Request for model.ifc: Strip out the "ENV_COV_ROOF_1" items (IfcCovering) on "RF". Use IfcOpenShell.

First a look at what the model holds.

```python
import ifcopenshell
import ifcopenshell.util.element

model = ifcopenshell.open("model.ifc")
print(model.schema)
storey = next(s for s in model.by_type("IfcBuildingStorey") if s.Name == "RF")
coverings = [e for e in ifcopenshell.util.element.get_decomposition(storey) if e.is_a("IfcCovering")]
seen = {}
for e in coverings:
    element_type = ifcopenshell.util.element.get_type(e)
    name = element_type.Name if element_type not in (None, e) else None
    seen[name] = seen.get(name, 0) + 1
for name, count in sorted(seen.items(), key=str):
    print(count, "x", name)
```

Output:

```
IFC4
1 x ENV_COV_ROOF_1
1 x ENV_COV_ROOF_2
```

```python
import ifcopenshell
import ifcopenshell.api.root
import ifcopenshell.util.element

model = ifcopenshell.open("model.ifc")

storey = next(s for s in model.by_type("IfcBuildingStorey") if s.Name == "RF")
coverings = [e for e in ifcopenshell.util.element.get_decomposition(storey) if e.is_a("IfcCovering")]
targets = [e for e in coverings if (t := ifcopenshell.util.element.get_type(e)) not in (None, e) and t.Name == "ENV_COV_ROOF_1"]

for e in targets:
    ifcopenshell.api.root.remove_product(model, product=e)
print(len(targets), "removed")

model.write("model_v2.ifc")
```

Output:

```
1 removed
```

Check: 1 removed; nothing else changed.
